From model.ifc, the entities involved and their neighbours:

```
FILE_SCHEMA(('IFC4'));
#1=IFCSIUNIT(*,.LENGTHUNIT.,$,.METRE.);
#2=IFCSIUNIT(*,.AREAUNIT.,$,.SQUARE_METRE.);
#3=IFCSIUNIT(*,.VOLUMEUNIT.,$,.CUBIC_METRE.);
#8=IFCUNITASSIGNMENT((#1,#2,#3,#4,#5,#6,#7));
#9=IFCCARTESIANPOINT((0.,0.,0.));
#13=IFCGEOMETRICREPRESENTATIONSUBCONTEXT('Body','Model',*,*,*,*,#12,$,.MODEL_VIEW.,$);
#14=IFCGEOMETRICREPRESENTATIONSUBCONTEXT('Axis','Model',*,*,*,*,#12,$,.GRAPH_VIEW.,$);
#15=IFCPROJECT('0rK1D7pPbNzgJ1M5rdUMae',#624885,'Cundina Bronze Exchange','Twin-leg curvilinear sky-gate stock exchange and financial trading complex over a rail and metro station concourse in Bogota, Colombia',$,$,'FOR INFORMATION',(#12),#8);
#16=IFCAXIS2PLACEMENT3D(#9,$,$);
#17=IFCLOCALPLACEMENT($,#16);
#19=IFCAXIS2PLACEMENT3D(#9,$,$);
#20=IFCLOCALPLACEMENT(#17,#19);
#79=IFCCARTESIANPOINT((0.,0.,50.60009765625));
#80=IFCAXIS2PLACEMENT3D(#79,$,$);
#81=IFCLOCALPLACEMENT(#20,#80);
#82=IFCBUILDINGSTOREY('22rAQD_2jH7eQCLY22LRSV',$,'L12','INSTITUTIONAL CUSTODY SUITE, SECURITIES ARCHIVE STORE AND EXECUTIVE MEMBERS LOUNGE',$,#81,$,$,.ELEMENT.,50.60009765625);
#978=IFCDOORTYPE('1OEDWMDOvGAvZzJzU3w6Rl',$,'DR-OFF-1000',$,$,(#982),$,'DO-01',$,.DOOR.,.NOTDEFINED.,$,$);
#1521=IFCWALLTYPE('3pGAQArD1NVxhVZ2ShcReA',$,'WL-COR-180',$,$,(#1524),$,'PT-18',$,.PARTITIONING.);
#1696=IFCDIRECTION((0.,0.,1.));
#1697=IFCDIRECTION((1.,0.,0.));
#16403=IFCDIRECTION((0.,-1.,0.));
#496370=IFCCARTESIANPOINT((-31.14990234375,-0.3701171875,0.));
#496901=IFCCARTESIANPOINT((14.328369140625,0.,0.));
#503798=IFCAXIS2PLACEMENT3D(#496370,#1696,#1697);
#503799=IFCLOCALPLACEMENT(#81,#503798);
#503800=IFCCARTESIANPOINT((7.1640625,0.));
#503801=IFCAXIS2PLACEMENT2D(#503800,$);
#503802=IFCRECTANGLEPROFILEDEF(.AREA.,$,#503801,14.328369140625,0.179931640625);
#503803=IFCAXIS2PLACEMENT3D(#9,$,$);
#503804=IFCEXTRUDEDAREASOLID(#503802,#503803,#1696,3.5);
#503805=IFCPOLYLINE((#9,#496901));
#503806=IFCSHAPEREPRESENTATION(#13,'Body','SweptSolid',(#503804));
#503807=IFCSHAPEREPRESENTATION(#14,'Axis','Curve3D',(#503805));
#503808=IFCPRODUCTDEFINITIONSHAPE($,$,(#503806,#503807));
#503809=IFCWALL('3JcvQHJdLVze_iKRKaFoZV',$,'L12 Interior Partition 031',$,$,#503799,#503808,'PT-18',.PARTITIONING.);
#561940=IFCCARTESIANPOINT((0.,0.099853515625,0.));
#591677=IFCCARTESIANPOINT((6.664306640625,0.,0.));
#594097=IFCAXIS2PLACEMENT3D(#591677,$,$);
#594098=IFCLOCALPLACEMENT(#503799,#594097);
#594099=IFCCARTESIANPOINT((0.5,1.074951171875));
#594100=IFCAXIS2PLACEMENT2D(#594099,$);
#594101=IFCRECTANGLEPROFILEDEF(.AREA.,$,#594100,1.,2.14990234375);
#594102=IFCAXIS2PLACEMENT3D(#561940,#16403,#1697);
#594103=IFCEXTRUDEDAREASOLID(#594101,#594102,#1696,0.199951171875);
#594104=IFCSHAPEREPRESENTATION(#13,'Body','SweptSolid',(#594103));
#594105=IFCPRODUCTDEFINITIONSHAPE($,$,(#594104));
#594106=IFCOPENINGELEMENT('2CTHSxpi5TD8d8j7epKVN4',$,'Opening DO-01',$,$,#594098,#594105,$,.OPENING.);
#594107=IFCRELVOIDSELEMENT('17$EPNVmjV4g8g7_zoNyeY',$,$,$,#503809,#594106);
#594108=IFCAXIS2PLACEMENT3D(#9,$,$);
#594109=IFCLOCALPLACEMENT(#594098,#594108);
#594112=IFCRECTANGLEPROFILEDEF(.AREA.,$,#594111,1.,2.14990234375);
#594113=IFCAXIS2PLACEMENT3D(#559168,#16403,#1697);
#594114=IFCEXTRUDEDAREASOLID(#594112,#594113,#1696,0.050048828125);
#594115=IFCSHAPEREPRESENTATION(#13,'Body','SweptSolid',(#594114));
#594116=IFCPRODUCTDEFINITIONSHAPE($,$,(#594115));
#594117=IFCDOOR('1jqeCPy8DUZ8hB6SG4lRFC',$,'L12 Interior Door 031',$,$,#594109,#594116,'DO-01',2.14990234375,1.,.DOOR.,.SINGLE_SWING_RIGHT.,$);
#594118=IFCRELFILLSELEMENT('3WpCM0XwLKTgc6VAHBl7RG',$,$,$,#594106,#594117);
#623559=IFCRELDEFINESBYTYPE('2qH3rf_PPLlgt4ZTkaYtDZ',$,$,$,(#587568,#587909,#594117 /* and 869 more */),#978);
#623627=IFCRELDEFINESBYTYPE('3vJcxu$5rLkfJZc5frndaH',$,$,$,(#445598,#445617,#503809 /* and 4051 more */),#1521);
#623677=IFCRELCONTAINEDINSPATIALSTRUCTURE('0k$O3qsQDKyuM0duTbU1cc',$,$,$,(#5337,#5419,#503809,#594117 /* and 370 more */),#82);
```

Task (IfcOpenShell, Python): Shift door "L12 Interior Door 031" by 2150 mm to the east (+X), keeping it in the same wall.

```python
import ifcopenshell
import ifcopenshell.api.geometry
import ifcopenshell.util.placement

model = ifcopenshell.open("model.ifc")

door = model.by_guid("1jqeCPy8DUZ8hB6SG4lRFC")
opening = door.FillsVoids[0].RelatingOpeningElement
wall = opening.VoidsElements[0].RelatingBuildingElement

wall_matrix = ifcopenshell.util.placement.get_local_placement(wall.ObjectPlacement)
shift = wall_matrix[:3, 0] * 2.15
before = ifcopenshell.util.placement.get_local_placement(door.ObjectPlacement)[:3, 3].copy()

# The door is placed relative to its opening, so it follows when the opening moves.
matrix = ifcopenshell.util.placement.get_local_placement(opening.ObjectPlacement)
matrix[:3, 3] += shift
ifcopenshell.api.geometry.edit_object_placement(
    model, product=opening, matrix=matrix, is_si=False, should_transform_children=True
)

after = ifcopenshell.util.placement.get_local_placement(door.ObjectPlacement)[:3, 3]
print("door moved by", (after - before).round(3) + 0.0)

model.write("model_updated.ifc")
```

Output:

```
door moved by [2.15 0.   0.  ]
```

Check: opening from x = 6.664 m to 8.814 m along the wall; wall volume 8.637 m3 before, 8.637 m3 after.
